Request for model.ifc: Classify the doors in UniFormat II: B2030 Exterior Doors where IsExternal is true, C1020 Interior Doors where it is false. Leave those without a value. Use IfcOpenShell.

First a look at what the model holds.

```python
import ifcopenshell
import ifcopenshell.util.element

model = ifcopenshell.open("model.ifc")
print(model.schema)
print("classifications:", [c.Name for c in model.by_type("IfcClassification")])
values = [ifcopenshell.util.element.get_pset(e, "Pset_DoorCommon", "IsExternal") for e in model.by_type("IfcDoor")]
for value in (True, False, None):
    print("IsExternal", value, values.count(value))
```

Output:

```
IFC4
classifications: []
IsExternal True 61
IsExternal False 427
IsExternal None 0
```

```python
import ifcopenshell
import ifcopenshell.api.classification
import ifcopenshell.util.element

model = ifcopenshell.open("model.ifc")

system = ifcopenshell.api.classification.add_classification(model, classification="UniFormat II")

doors = model.by_type("IfcDoor")
external = {e: ifcopenshell.util.element.get_pset(e, "Pset_DoorCommon", "IsExternal") for e in doors}
for flag, code, name in ((True, "B2030", "Exterior Doors"), (False, "C1020", "Interior Doors")):
    products = [e for e in doors if external[e] is flag]
    ifcopenshell.api.classification.add_reference(
        model, products=products, classification=system, identification=code, name=name
    )
    print(code, len(products))

model.write("model-out.ifc")
```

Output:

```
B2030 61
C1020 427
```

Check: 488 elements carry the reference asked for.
